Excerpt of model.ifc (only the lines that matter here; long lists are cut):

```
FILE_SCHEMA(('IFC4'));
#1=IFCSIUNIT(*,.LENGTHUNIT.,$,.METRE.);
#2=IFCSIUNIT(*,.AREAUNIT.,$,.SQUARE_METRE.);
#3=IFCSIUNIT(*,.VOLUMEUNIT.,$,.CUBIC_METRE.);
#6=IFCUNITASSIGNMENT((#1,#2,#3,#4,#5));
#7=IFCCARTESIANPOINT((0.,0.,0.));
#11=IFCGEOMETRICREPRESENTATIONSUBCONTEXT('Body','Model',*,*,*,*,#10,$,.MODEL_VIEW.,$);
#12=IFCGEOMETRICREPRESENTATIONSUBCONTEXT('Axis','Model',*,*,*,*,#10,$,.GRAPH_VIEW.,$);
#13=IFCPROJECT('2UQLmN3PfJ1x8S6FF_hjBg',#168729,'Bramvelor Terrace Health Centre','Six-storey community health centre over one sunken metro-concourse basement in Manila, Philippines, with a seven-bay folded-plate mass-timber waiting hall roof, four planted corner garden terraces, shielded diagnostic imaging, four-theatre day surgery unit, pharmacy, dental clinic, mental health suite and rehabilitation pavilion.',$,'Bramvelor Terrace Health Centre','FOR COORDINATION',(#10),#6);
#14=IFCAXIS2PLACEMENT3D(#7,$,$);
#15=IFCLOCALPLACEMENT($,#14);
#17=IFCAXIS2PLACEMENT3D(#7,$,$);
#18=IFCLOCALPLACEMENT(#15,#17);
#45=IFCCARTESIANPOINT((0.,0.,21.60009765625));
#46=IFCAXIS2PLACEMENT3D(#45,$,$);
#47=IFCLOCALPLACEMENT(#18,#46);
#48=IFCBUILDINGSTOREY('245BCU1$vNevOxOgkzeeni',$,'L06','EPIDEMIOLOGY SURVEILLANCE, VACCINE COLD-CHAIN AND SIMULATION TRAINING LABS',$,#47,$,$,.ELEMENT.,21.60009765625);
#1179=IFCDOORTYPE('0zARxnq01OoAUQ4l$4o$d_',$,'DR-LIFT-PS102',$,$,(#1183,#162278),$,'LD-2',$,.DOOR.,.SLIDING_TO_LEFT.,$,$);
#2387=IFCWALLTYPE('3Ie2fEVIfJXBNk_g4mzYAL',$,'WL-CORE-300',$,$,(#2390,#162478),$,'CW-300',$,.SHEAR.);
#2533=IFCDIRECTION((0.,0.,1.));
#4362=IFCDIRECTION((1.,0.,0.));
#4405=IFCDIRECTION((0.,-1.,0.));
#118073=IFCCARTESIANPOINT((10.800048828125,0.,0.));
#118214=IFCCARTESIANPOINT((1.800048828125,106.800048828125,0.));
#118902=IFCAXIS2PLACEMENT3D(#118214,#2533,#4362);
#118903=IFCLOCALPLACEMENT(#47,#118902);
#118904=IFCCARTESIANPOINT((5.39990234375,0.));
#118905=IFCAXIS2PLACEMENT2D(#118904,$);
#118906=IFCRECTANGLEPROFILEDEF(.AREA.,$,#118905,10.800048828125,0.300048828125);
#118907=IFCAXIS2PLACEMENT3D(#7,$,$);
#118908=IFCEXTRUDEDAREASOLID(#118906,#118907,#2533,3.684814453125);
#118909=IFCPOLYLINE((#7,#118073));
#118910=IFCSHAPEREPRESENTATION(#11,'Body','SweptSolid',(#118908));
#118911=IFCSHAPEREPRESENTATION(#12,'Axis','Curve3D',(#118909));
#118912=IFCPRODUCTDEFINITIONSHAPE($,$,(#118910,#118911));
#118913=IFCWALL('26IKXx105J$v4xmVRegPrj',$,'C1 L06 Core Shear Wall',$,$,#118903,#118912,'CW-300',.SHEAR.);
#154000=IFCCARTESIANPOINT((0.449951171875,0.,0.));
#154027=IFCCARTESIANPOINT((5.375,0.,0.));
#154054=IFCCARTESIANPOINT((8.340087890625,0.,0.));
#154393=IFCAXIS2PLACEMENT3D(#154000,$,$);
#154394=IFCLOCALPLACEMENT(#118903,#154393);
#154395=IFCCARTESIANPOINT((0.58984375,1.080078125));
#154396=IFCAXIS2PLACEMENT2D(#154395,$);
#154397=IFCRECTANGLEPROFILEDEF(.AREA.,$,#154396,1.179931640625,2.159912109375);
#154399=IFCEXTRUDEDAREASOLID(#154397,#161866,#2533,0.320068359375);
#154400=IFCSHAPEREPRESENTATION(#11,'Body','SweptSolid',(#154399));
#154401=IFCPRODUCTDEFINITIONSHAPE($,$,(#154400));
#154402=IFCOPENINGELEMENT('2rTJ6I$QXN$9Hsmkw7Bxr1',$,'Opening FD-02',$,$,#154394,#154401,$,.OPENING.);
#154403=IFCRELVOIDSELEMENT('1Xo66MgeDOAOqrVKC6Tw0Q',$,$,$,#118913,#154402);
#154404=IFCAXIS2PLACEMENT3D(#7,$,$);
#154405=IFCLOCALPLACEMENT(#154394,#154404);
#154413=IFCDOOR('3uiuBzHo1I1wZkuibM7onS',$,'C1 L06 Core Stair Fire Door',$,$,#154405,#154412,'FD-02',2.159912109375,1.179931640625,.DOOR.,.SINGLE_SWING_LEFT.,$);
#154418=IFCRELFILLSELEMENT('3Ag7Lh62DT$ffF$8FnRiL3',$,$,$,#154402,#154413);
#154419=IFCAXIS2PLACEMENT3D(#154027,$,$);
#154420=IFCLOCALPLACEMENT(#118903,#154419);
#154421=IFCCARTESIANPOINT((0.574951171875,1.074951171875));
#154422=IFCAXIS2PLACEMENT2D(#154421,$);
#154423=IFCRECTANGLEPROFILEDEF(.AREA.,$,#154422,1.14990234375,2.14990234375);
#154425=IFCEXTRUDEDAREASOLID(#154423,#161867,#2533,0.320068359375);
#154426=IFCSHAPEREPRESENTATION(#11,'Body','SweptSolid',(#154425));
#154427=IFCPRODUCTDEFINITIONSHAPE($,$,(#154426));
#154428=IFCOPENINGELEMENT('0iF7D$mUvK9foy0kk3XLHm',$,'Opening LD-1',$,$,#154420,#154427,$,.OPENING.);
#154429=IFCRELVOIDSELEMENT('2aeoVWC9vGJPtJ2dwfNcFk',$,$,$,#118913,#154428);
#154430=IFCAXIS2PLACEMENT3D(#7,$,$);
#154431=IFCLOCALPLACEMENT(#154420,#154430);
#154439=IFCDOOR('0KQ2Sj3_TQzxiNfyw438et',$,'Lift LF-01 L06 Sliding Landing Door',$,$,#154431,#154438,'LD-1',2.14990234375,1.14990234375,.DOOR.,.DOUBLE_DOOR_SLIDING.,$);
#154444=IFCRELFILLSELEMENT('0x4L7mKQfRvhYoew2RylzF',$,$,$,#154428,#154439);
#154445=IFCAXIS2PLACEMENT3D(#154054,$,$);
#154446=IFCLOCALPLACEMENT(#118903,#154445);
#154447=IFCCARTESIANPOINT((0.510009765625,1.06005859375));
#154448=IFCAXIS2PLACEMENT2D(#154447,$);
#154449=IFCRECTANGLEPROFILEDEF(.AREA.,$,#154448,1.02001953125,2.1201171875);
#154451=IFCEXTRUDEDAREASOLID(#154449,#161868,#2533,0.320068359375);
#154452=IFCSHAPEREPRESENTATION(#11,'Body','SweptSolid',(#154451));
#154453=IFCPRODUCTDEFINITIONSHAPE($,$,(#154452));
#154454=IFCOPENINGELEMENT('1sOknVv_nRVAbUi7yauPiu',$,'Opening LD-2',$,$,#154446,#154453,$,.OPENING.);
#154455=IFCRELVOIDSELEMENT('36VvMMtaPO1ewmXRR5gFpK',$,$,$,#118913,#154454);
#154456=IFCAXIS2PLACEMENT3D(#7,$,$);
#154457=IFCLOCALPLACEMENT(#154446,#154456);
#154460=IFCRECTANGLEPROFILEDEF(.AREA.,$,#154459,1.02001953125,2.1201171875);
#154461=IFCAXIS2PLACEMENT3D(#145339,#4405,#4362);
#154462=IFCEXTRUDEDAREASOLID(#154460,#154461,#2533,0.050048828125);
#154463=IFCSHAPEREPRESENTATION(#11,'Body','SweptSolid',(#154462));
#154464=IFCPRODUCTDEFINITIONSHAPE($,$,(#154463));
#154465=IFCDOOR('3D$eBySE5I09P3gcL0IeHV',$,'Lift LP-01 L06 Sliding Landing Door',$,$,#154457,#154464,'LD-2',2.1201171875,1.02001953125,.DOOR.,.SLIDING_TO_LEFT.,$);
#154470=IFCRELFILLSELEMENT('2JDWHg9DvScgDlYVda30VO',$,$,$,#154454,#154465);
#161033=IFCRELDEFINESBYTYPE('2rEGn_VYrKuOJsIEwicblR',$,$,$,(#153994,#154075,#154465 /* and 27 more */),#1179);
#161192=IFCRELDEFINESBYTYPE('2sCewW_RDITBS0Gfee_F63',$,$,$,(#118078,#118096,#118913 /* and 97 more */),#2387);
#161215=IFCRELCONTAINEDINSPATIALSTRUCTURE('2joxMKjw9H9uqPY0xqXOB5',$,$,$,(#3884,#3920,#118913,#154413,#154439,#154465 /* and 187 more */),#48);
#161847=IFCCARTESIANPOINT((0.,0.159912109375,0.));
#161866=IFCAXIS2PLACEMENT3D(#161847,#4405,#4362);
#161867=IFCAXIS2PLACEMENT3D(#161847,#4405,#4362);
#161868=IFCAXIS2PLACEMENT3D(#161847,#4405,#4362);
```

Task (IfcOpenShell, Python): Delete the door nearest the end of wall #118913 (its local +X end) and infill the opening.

```python
import ifcopenshell
import ifcopenshell.api.feature
import ifcopenshell.api.root
import ifcopenshell.geom
import ifcopenshell.util.shape

model = ifcopenshell.open("model.ifc")
settings = ifcopenshell.geom.settings()


def volume(element):
    """Net volume in cubic metres, openings subtracted."""
    shape = ifcopenshell.geom.create_shape(settings, element)
    return ifcopenshell.util.shape.get_volume(shape.geometry)


door = model.by_guid("3D$eBySE5I09P3gcL0IeHV")
opening = door.FillsVoids[0].RelatingOpeningElement
wall = opening.VoidsElements[0].RelatingBuildingElement
before = volume(wall)

ifcopenshell.api.root.remove_product(model, product=door)
ifcopenshell.api.feature.remove_feature(model, feature=opening)

after = volume(wall)

print(f"wall volume {before:.3f} -> {after:.3f} m3")

model.write("model_v2.ifc")
```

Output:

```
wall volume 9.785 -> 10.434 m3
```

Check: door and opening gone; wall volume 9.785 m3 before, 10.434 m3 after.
